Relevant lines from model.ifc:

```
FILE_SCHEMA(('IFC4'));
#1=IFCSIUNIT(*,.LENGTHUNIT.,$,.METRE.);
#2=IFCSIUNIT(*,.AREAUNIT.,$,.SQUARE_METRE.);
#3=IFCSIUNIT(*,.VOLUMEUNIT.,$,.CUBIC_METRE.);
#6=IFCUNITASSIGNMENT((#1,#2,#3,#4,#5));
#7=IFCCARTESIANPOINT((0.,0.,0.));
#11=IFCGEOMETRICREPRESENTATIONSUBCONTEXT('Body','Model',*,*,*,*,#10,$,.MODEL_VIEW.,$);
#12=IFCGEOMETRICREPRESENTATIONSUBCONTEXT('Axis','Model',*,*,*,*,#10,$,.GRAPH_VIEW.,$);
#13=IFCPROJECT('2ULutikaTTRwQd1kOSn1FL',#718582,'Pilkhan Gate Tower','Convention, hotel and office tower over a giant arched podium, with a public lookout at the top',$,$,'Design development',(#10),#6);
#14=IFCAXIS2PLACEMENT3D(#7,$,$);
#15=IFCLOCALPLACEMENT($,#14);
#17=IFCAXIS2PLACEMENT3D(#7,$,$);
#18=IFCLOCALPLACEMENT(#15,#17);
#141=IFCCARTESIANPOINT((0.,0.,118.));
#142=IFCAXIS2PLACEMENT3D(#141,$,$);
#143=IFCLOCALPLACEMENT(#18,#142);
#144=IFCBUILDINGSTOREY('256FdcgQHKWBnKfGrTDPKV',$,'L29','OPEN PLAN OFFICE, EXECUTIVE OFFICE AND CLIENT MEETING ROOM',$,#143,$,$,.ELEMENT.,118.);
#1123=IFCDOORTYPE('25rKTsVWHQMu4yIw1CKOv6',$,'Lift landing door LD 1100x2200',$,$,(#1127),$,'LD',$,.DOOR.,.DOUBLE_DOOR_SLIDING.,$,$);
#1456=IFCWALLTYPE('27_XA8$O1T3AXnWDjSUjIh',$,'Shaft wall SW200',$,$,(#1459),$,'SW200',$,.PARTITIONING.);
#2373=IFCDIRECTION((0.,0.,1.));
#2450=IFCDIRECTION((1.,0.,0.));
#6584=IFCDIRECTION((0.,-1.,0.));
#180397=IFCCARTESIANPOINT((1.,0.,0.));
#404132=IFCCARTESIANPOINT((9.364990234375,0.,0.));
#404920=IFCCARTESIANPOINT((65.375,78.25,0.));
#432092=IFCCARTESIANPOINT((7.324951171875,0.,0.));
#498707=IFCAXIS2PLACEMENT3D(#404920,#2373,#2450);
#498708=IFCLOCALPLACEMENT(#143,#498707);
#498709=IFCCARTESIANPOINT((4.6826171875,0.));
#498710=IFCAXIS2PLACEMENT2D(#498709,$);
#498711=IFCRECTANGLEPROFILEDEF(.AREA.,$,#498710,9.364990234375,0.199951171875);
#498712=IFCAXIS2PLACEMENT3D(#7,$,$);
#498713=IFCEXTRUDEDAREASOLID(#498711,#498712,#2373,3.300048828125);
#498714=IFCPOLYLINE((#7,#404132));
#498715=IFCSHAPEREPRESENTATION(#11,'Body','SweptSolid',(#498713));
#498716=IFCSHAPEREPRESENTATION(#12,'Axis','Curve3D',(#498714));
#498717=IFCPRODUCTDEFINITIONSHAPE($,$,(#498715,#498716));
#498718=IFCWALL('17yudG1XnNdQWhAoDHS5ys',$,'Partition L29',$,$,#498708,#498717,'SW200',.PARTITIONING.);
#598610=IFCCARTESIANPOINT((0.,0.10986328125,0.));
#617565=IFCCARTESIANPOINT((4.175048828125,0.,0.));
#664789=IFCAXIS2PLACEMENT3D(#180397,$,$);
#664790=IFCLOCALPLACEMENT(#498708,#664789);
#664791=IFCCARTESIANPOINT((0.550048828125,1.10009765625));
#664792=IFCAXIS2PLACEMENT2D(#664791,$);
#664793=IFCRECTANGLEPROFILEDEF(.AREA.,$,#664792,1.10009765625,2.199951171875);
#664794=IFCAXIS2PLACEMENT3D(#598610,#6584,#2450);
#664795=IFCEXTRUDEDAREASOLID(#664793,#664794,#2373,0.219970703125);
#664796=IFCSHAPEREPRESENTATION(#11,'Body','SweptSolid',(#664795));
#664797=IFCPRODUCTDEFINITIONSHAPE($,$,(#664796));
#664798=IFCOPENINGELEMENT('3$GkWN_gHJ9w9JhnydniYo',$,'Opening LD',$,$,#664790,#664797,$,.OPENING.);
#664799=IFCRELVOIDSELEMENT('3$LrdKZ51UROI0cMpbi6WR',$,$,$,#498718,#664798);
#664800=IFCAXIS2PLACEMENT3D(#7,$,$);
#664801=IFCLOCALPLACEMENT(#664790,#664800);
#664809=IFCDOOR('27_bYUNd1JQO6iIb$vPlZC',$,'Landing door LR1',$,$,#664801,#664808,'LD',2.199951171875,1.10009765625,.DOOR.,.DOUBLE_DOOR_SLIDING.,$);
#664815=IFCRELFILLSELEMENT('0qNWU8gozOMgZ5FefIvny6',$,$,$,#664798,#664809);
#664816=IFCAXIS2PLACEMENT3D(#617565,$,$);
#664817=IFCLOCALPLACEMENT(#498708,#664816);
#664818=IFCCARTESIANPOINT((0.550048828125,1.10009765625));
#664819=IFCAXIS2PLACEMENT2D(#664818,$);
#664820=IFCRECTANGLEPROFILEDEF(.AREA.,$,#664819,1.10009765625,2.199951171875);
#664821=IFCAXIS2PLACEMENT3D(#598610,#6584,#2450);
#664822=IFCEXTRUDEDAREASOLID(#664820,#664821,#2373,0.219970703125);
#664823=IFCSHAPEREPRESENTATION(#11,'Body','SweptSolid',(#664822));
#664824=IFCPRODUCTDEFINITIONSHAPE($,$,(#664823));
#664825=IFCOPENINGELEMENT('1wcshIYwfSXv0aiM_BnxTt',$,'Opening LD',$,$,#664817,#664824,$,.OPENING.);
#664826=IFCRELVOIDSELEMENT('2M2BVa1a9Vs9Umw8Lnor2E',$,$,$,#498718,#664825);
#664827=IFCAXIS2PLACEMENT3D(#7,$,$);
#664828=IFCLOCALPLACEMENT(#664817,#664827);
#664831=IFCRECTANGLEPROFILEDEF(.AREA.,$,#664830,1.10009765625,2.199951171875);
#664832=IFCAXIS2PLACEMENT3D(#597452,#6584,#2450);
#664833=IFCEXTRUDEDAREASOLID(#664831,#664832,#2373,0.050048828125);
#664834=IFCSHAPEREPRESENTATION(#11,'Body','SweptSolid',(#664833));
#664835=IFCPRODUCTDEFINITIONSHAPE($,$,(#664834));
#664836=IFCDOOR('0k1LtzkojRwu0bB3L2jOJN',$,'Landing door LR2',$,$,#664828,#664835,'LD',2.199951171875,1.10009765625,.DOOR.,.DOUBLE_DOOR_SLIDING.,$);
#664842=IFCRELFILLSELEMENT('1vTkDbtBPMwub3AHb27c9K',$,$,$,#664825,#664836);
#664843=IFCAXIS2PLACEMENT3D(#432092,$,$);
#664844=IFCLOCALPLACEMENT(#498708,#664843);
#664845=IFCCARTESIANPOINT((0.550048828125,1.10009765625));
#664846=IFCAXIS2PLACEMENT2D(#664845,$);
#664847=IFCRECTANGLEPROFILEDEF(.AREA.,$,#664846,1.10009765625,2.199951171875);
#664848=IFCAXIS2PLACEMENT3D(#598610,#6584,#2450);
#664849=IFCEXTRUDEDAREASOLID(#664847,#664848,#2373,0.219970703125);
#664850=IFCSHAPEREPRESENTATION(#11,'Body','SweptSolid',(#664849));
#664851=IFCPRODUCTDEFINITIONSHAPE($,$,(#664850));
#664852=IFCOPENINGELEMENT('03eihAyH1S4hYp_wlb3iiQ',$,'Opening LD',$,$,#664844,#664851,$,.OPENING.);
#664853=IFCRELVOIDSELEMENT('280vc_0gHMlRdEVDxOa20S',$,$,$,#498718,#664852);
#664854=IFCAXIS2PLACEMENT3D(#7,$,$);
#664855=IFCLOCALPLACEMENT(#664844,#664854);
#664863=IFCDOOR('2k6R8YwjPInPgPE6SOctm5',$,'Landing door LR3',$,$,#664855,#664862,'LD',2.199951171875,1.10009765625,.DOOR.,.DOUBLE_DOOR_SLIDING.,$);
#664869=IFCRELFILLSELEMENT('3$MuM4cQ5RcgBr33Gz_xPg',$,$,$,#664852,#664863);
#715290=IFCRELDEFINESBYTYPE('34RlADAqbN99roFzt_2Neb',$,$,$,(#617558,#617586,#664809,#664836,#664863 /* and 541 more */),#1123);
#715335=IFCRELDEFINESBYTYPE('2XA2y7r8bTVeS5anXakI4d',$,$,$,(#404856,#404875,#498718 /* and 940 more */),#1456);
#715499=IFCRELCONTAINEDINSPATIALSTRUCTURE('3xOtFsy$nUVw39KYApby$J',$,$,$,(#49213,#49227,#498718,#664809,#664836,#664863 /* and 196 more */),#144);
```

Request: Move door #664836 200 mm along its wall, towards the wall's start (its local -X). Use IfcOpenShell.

```python
import ifcopenshell
import ifcopenshell.api.geometry
import ifcopenshell.util.placement
import ifcopenshell.util.unit

model = ifcopenshell.open("model.ifc")
unit_scale = ifcopenshell.util.unit.calculate_unit_scale(model)

door = model.by_guid("0k1LtzkojRwu0bB3L2jOJN")
opening = door.FillsVoids[0].RelatingOpeningElement
wall = opening.VoidsElements[0].RelatingBuildingElement

wall_matrix = ifcopenshell.util.placement.get_local_placement(wall.ObjectPlacement)
shift = wall_matrix[:3, 0] * -0.2 / unit_scale
before = ifcopenshell.util.placement.get_local_placement(door.ObjectPlacement)[:3, 3].copy()

# The door is placed relative to its opening, so it follows when the opening moves.
matrix = ifcopenshell.util.placement.get_local_placement(opening.ObjectPlacement)
matrix[:3, 3] += shift
ifcopenshell.api.geometry.edit_object_placement(
    model, product=opening, matrix=matrix, is_si=False, should_transform_children=True
)

after = ifcopenshell.util.placement.get_local_placement(door.ObjectPlacement)[:3, 3]
print("door moved by", (after - before).round(3) + 0.0)

model.write("model_updated.ifc")
```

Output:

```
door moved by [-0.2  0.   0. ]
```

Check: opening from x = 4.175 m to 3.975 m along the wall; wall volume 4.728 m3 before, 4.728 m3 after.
